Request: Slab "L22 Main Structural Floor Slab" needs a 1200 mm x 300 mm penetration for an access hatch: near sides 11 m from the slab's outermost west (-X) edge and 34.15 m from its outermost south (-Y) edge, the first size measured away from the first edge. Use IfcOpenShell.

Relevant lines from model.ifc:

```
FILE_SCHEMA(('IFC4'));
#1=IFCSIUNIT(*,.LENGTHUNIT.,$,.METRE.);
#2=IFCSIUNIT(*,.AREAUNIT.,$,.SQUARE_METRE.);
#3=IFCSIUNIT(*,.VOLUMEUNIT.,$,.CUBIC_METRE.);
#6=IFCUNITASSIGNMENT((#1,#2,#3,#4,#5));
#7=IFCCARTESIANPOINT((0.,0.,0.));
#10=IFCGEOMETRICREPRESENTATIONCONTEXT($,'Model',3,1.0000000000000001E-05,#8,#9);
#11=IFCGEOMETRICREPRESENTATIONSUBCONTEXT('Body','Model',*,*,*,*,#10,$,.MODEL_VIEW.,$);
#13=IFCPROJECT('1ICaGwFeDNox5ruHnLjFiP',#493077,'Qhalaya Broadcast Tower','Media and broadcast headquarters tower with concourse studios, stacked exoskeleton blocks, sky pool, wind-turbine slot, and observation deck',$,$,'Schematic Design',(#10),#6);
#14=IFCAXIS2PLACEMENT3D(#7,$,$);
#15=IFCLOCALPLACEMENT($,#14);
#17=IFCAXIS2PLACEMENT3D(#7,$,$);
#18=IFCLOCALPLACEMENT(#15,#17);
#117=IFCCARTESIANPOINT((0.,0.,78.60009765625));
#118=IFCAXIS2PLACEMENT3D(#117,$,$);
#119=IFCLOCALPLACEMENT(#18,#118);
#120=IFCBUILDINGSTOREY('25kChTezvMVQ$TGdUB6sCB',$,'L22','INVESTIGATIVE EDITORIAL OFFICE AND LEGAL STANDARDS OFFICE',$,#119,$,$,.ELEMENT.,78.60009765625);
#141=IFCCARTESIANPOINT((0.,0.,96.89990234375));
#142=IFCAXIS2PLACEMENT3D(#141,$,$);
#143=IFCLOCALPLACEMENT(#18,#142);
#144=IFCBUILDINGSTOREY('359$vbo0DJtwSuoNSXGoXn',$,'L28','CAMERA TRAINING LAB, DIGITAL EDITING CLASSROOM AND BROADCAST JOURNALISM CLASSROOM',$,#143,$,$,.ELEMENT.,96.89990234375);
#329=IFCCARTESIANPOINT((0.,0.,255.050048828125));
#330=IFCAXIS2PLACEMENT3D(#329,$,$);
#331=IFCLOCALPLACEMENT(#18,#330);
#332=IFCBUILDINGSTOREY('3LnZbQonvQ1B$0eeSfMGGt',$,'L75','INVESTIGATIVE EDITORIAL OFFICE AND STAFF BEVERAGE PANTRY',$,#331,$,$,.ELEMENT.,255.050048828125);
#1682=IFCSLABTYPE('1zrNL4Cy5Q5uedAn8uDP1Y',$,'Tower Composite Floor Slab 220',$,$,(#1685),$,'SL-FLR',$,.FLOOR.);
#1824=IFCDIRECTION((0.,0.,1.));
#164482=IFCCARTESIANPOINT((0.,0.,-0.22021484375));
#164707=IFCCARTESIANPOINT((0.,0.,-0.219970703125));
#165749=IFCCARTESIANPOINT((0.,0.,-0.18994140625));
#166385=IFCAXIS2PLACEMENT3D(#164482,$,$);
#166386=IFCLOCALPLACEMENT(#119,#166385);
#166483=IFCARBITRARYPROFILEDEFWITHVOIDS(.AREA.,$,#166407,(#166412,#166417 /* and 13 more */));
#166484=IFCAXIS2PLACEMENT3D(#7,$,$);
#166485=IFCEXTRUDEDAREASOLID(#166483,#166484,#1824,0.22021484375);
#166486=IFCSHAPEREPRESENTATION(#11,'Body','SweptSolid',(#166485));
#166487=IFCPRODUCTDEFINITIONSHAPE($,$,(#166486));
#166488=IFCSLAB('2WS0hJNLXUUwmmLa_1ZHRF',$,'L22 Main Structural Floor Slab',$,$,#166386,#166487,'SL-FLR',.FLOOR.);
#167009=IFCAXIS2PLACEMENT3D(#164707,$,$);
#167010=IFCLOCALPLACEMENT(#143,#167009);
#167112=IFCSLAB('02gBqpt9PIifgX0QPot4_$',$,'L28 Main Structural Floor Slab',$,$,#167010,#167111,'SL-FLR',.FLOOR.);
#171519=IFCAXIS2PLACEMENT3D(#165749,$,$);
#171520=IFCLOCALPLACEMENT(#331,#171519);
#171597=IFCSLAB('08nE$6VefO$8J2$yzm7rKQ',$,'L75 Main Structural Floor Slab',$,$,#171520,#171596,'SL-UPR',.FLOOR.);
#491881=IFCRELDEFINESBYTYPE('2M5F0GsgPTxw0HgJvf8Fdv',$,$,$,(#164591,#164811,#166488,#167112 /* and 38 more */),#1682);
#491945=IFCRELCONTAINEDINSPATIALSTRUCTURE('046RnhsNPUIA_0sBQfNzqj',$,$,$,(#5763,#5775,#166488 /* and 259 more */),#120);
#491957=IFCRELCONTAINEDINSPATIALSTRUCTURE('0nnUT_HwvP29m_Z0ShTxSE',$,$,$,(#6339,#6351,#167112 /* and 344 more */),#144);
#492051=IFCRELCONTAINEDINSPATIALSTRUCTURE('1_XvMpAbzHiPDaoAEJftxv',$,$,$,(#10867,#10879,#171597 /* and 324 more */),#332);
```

```python
import numpy as np
import ifcopenshell
import ifcopenshell.api.feature
import ifcopenshell.api.geometry
import ifcopenshell.api.root
import ifcopenshell.geom
import ifcopenshell.util.placement
import ifcopenshell.util.representation
import ifcopenshell.util.shape
import ifcopenshell.util.unit

model = ifcopenshell.open("model.ifc")
unit_scale = ifcopenshell.util.unit.calculate_unit_scale(model)
settings = ifcopenshell.geom.settings()


def volume(element):
    """Net volume in cubic metres, openings subtracted."""
    shape = ifcopenshell.geom.create_shape(settings, element)
    return ifcopenshell.util.shape.get_volume(shape.geometry)


slab = model.by_id(166488)
before = volume(slab)

# Extent in the slab's own axes, in metres. The edges named are its -X and -Y sides.
slab_shape = ifcopenshell.geom.create_shape(settings, slab)
vertices = ifcopenshell.util.shape.get_vertices(slab_shape.geometry)
x_min, y_min, bottom = vertices.min(axis=0)
top = vertices[:, 2].max()

opening = ifcopenshell.api.root.create_entity(model, ifc_class="IfcOpeningElement", name="Access hatch opening", predefined_type="OPENING")
context = ifcopenshell.util.representation.get_context(model, "Model", "Body", "MODEL_VIEW")
width, depth = 1.2, 0.3
outline = [(0.0, 0.0), (width, 0.0), (width, depth), (0.0, depth), (0.0, 0.0)]
# Overshoot both faces by 50 mm so the cut is clean.
shape = ifcopenshell.api.geometry.add_slab_representation(
    model, context=context, depth=top - bottom + 0.1, polyline=outline
)
ifcopenshell.api.geometry.assign_representation(model, product=opening, representation=shape)

matrix = ifcopenshell.util.placement.get_local_placement(slab.ObjectPlacement)
matrix[:, 3] = matrix @ np.append(np.array([x_min + 11, y_min + 34.15, bottom - 0.05]) / unit_scale, 1.0)
ifcopenshell.api.geometry.edit_object_placement(model, product=opening, matrix=matrix, is_si=False)
ifcopenshell.api.feature.add_feature(model, feature=opening, element=slab)

after = volume(slab)

print(f"slab volume {before:.3f} -> {after:.3f} m3")

model.write("model_rev.ifc")
```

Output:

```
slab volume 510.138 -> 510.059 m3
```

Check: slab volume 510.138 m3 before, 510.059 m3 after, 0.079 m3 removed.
